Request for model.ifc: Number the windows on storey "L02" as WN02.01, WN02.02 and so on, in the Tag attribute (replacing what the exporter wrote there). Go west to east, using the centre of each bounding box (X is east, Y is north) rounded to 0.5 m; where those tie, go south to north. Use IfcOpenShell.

First a look at what the model holds.

```python
import ifcopenshell
import ifcopenshell.util.element
import ifcopenshell.util.placement

model = ifcopenshell.open("model.ifc")
print(model.schema)
storey = next(s for s in model.by_type("IfcBuildingStorey") if s.Name == "L02")
windows = [e for e in ifcopenshell.util.element.get_decomposition(storey) if e.is_a("IfcWindow")]
for e in sorted(windows, key=lambda e: e.id()):
    origin = ifcopenshell.util.placement.get_local_placement(e.ObjectPlacement)[:3, 3]
    print(e.id(), e.Tag, e.Name, origin.round(2) + 0.0, sep=" | ")
```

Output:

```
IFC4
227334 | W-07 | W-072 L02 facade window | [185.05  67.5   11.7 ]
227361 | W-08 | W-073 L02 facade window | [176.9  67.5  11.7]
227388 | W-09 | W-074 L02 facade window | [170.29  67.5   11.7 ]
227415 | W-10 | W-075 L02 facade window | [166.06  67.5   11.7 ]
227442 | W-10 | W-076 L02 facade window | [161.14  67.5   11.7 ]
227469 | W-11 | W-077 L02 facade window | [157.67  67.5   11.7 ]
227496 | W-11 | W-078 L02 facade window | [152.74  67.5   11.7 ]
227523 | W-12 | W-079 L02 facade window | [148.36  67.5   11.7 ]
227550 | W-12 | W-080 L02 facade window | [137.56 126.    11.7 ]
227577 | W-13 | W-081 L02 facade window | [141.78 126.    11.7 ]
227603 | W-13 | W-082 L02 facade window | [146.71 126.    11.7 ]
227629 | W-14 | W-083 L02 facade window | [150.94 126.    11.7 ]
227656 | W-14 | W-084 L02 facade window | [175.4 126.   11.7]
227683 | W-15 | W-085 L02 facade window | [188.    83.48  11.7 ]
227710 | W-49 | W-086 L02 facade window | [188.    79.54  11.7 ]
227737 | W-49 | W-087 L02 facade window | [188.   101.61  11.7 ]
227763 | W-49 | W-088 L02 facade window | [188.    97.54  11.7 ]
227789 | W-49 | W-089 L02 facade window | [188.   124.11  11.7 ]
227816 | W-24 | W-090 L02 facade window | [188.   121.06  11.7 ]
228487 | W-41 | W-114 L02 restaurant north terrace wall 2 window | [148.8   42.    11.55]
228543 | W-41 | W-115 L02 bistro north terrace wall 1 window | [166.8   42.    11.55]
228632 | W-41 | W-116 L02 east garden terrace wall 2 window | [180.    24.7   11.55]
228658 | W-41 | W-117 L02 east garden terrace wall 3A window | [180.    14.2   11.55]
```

```python
import ifcopenshell
import ifcopenshell.geom
import ifcopenshell.util.element
import ifcopenshell.util.shape

model = ifcopenshell.open("model.ifc")
settings = ifcopenshell.geom.settings()
settings.set("use-world-coords", True)


def centre(element):
    shape = ifcopenshell.geom.create_shape(settings, element)
    return ifcopenshell.util.shape.get_bbox_centroid(shape.geometry)


storey = next(s for s in model.by_type("IfcBuildingStorey") if s.Name == "L02")
windows = [e for e in ifcopenshell.util.element.get_decomposition(storey) if e.is_a("IfcWindow")]

# Insertion points can sit at a corner or the storey origin, so sort by the geometry (in metres).
centres = {e: centre(e) for e in windows}
windows.sort(key=lambda e: (round(centres[e][0] / 0.5), centres[e][1]))

for i, e in enumerate(windows, start=1):
    number = f"WN02.{i:02d}"
    e.Tag = number
    print(e.id(), number)

model.write("model_edited.ifc")
```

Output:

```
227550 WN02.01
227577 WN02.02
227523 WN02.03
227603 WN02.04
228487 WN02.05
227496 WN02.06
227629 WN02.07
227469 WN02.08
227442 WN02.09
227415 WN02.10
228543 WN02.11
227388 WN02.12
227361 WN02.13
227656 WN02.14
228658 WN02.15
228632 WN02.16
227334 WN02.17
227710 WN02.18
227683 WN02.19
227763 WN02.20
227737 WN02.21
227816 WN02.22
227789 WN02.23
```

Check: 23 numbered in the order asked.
